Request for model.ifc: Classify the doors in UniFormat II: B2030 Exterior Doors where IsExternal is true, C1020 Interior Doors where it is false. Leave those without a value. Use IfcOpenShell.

First a look at what the model holds.

```python
import ifcopenshell
import ifcopenshell.util.element

model = ifcopenshell.open("model.ifc")
print(model.schema)
print("classifications:", [c.Name for c in model.by_type("IfcClassification")])
values = [ifcopenshell.util.element.get_pset(e, "Pset_DoorCommon", "IsExternal") for e in model.by_type("IfcDoor")]
for value in (True, False, None):
    print("IsExternal", value, values.count(value))
```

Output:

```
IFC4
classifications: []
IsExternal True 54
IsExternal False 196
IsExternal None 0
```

```python
import ifcopenshell
import ifcopenshell.api.classification
import ifcopenshell.util.element

model = ifcopenshell.open("model.ifc")

system = ifcopenshell.api.classification.add_classification(model, classification="UniFormat II")

doors = model.by_type("IfcDoor")
external = {e: ifcopenshell.util.element.get_pset(e, "Pset_DoorCommon", "IsExternal") for e in doors}
for flag, code, name in ((True, "B2030", "Exterior Doors"), (False, "C1020", "Interior Doors")):
    products = [e for e in doors if external[e] is flag]
    ifcopenshell.api.classification.add_reference(
        model, products=products, classification=system, identification=code, name=name
    )
    print(code, len(products))

model.write("model-out.ifc")
```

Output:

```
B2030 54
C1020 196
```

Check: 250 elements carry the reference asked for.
